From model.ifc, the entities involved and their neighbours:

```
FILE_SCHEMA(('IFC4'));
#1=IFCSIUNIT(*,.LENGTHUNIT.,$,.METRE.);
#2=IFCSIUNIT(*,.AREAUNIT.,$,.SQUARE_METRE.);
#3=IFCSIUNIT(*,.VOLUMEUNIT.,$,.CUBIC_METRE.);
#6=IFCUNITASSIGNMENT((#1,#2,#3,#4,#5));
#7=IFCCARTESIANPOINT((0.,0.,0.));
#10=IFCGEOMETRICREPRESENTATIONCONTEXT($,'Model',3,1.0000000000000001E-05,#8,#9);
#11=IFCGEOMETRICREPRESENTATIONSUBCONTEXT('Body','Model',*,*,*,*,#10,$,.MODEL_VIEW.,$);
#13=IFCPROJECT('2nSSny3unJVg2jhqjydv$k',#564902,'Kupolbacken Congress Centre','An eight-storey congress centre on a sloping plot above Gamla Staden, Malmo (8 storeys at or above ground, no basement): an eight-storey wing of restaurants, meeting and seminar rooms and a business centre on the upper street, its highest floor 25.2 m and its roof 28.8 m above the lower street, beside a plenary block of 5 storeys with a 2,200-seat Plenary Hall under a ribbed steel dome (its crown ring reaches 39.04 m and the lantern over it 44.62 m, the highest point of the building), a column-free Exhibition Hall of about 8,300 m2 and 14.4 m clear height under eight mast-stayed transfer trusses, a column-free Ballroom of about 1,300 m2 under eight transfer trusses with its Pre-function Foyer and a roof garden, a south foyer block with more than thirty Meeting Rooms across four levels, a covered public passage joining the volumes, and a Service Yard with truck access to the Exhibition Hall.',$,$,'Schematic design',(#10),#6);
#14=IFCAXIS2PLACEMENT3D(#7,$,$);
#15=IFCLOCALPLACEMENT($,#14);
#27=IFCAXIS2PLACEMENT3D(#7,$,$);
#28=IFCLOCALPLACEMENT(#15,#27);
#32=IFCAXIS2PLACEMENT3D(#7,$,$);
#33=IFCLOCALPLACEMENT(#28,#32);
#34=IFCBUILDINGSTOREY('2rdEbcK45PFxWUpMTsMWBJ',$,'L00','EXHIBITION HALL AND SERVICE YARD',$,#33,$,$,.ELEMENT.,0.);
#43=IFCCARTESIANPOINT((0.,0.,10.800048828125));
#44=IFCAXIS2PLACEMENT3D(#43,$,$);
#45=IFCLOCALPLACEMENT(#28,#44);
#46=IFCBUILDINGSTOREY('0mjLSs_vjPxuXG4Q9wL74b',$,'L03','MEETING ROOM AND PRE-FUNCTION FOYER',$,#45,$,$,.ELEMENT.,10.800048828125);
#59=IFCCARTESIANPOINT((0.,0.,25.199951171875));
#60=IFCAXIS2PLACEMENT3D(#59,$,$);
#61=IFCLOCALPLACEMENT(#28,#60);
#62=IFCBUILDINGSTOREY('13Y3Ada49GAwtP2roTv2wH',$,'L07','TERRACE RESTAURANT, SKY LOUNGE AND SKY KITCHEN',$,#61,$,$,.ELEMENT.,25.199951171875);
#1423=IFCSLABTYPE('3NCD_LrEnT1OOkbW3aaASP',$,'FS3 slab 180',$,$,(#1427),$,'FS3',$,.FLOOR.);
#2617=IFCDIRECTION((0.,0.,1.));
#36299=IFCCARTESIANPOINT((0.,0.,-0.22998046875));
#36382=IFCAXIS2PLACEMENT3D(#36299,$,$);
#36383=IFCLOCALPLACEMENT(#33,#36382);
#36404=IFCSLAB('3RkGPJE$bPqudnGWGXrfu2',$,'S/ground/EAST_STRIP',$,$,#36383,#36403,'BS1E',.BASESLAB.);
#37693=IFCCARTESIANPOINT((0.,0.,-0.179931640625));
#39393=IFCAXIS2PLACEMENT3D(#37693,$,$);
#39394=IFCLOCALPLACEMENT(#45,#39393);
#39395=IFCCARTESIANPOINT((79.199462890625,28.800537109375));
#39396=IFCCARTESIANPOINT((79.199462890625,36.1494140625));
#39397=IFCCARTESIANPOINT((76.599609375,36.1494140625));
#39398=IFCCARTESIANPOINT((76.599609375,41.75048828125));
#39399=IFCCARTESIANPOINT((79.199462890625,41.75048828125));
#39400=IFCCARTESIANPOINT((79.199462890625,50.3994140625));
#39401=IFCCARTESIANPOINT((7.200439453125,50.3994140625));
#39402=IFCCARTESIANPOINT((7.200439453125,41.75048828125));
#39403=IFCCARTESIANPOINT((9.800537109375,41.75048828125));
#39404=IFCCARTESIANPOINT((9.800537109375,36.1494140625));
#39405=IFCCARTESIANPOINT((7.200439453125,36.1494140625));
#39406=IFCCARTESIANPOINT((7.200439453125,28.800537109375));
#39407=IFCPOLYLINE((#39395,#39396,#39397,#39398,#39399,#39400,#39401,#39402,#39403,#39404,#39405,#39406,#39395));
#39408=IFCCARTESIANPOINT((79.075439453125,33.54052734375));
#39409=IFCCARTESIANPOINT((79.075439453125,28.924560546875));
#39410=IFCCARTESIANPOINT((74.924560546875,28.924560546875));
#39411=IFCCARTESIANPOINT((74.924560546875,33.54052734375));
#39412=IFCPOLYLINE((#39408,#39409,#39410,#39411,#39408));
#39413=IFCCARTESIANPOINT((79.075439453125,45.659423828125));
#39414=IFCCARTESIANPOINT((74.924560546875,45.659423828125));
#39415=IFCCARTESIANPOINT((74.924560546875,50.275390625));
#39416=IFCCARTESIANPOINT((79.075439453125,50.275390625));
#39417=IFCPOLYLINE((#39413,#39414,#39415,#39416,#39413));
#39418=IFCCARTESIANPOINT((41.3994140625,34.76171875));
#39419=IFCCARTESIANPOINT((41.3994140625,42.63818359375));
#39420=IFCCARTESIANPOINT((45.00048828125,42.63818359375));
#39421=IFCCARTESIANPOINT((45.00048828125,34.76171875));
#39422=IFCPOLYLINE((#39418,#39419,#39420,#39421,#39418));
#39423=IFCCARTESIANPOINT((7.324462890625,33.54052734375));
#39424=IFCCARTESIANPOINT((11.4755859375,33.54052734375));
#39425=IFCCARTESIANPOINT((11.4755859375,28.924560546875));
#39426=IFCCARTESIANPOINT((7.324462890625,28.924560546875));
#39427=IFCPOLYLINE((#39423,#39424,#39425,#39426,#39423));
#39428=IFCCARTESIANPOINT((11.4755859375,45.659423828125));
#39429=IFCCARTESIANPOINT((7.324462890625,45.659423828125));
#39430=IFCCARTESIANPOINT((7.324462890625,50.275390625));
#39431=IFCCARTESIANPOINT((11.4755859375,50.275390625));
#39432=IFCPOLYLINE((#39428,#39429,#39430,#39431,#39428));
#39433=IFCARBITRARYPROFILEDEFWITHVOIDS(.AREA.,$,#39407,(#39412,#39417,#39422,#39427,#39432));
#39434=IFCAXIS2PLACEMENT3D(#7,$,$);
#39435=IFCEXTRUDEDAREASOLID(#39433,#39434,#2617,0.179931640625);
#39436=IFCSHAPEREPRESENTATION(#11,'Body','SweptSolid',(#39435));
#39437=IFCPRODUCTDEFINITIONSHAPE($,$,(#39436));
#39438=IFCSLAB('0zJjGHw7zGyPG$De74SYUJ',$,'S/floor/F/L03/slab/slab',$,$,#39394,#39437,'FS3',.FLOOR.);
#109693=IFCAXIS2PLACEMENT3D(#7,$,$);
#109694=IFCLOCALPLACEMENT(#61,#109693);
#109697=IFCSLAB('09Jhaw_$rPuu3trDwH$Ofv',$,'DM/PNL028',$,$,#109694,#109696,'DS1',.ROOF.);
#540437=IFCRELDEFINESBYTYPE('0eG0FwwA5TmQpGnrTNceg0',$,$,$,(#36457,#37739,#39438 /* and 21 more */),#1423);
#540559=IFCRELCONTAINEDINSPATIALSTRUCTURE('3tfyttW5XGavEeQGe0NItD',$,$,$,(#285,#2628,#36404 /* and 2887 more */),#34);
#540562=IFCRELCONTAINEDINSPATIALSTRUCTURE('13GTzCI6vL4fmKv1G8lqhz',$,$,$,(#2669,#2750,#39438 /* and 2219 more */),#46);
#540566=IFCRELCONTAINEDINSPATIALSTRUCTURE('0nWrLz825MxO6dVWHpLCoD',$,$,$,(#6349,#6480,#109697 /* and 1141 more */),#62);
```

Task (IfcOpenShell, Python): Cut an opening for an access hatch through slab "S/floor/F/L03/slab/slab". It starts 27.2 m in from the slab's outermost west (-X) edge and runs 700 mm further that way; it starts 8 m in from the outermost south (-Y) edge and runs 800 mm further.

```python
import numpy as np
import ifcopenshell
import ifcopenshell.api.feature
import ifcopenshell.api.geometry
import ifcopenshell.api.root
import ifcopenshell.geom
import ifcopenshell.util.placement
import ifcopenshell.util.representation
import ifcopenshell.util.shape
import ifcopenshell.util.unit

model = ifcopenshell.open("model.ifc")
unit_scale = ifcopenshell.util.unit.calculate_unit_scale(model)
settings = ifcopenshell.geom.settings()


def volume(element):
    """Net volume in cubic metres, openings subtracted."""
    shape = ifcopenshell.geom.create_shape(settings, element)
    return ifcopenshell.util.shape.get_volume(shape.geometry)


slab = model.by_id(39438)
before = volume(slab)

# Extent in the slab's own axes, in metres. The edges named are its -X and -Y sides.
slab_shape = ifcopenshell.geom.create_shape(settings, slab)
vertices = ifcopenshell.util.shape.get_vertices(slab_shape.geometry)
x_min, y_min, bottom = vertices.min(axis=0)
top = vertices[:, 2].max()

opening = ifcopenshell.api.root.create_entity(model, ifc_class="IfcOpeningElement", name="Access hatch opening", predefined_type="OPENING")
context = ifcopenshell.util.representation.get_context(model, "Model", "Body", "MODEL_VIEW")
width, depth = 0.7, 0.8
outline = [(0.0, 0.0), (width, 0.0), (width, depth), (0.0, depth), (0.0, 0.0)]
# Overshoot both faces by 50 mm so the cut is clean.
shape = ifcopenshell.api.geometry.add_slab_representation(
    model, context=context, depth=top - bottom + 0.1, polyline=outline
)
ifcopenshell.api.geometry.assign_representation(model, product=opening, representation=shape)

matrix = ifcopenshell.util.placement.get_local_placement(slab.ObjectPlacement)
matrix[:, 3] = matrix @ np.append(np.array([x_min + 27.2, y_min + 8, bottom - 0.05]) / unit_scale, 1.0)
ifcopenshell.api.geometry.edit_object_placement(model, product=opening, matrix=matrix, is_si=False)
ifcopenshell.api.feature.add_feature(model, feature=opening, element=slab)

after = volume(slab)

print(f"slab volume {before:.3f} -> {after:.3f} m3")

model.write("model_v2.ifc")
```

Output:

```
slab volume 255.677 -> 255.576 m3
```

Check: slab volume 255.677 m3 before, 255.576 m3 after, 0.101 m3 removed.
